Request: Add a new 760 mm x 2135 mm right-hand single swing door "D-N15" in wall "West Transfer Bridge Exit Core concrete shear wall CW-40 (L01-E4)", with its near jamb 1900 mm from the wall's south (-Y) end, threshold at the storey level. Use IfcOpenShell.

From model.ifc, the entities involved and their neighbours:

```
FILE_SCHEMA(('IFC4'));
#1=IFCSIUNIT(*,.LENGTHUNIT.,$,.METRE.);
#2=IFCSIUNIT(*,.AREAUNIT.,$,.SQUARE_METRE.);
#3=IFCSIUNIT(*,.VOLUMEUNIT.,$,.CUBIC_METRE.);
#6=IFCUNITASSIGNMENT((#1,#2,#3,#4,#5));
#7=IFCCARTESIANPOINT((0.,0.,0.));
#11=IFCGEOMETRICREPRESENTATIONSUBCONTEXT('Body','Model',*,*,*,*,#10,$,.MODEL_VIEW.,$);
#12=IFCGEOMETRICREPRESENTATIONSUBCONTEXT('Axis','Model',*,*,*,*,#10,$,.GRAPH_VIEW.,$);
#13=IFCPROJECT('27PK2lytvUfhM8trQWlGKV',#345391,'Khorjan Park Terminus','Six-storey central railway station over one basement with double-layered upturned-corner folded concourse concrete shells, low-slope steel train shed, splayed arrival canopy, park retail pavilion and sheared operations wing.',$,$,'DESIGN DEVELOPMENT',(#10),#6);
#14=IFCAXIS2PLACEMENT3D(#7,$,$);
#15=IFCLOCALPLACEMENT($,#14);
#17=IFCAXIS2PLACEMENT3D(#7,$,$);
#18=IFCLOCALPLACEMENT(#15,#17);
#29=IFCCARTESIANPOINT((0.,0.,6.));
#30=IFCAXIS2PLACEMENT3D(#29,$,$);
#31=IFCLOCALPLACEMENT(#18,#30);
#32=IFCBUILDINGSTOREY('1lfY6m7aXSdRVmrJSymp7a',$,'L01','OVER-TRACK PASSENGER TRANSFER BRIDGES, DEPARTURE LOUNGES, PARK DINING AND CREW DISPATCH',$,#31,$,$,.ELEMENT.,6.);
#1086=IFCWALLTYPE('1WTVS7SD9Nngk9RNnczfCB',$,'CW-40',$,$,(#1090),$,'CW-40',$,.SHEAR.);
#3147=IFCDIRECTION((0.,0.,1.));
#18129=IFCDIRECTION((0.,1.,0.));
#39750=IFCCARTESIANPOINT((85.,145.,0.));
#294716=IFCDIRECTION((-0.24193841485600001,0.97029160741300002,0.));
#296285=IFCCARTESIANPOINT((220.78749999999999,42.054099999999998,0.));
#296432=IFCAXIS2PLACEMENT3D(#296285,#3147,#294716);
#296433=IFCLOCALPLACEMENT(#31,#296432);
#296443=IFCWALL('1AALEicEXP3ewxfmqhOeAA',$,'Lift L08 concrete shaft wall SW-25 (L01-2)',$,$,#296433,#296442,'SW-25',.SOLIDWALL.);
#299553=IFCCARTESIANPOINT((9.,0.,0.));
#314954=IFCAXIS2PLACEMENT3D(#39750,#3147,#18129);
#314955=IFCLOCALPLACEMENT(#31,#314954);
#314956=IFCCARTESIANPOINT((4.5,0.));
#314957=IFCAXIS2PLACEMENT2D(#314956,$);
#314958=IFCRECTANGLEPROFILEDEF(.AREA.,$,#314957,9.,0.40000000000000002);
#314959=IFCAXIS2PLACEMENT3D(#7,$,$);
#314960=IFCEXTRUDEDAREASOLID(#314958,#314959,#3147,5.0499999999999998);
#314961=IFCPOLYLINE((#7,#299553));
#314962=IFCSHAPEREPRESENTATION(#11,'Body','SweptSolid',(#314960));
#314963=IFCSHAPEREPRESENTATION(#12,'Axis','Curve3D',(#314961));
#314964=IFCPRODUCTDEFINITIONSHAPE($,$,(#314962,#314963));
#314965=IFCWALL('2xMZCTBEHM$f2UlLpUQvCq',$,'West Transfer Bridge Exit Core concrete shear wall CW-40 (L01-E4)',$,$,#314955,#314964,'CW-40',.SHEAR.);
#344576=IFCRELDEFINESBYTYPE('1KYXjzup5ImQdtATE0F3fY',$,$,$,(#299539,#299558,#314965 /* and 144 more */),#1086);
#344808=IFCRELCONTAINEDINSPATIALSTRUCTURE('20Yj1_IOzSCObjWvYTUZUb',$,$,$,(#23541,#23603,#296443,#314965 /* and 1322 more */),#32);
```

```python
import numpy as np
import ifcopenshell
import ifcopenshell.api.feature
import ifcopenshell.api.geometry
import ifcopenshell.api.root
import ifcopenshell.api.spatial
import ifcopenshell.geom
import ifcopenshell.util.element
import ifcopenshell.util.placement
import ifcopenshell.util.representation
import ifcopenshell.util.shape
import ifcopenshell.util.unit

model = ifcopenshell.open("model.ifc")
unit_scale = ifcopenshell.util.unit.calculate_unit_scale(model)
settings = ifcopenshell.geom.settings()


def volume(element):
    """Net volume in cubic metres, openings subtracted."""
    shape = ifcopenshell.geom.create_shape(settings, element)
    return ifcopenshell.util.shape.get_volume(shape.geometry)


wall = model.by_guid("2xMZCTBEHM$f2UlLpUQvCq")
storey = ifcopenshell.util.element.get_container(wall, ifc_class="IfcBuildingStorey")
context = ifcopenshell.util.representation.get_context(model, "Model", "Body", "MODEL_VIEW")
before = volume(wall)

width, height, from_end, sill = 0.76, 2.135, 1.9, 0.0  # metres

# The wall runs along its own X axis, and the end named is its -X end.
wall_shape = ifcopenshell.geom.create_shape(settings, wall)
x, y, z = ifcopenshell.util.shape.get_vertices(wall_shape.geometry).T
start = x.min() + from_end
face, thickness = float(y.min()), float(y.max() - y.min())
wall_matrix = ifcopenshell.util.placement.get_local_placement(wall.ObjectPlacement)
level = ifcopenshell.util.placement.get_local_placement(storey.ObjectPlacement)[2, 3]


def in_wall(x, y):
    """Placement at x, y metres in the wall's axes, at sill height."""
    matrix = wall_matrix.copy()
    matrix[:, 3] = wall_matrix @ np.array([x / unit_scale, y / unit_scale, 0.0, 1.0])
    matrix[2, 3] = level + sill / unit_scale
    return matrix


# Opening: a box that overshoots both wall faces by 50 mm.
opening = ifcopenshell.api.root.create_entity(model, ifc_class="IfcOpeningElement", predefined_type="OPENING")
box = ifcopenshell.api.geometry.add_wall_representation(
    model, context=context, length=width, height=height, thickness=thickness + 0.1
)
ifcopenshell.api.geometry.assign_representation(model, product=opening, representation=box)
ifcopenshell.api.geometry.edit_object_placement(model, product=opening, matrix=in_wall(start, face - 0.05), is_si=False)
ifcopenshell.api.feature.add_feature(model, feature=opening, element=wall)

door = ifcopenshell.api.root.create_entity(model, ifc_class="IfcDoor", name="D-N15", predefined_type="DOOR")
door.OverallWidth, door.OverallHeight = width / unit_scale, height / unit_scale
door.OperationType = "SINGLE_SWING_RIGHT"
body = ifcopenshell.api.geometry.add_door_representation(
    model,
    context=context,
    overall_width=door.OverallWidth,
    overall_height=door.OverallHeight,
    operation_type="SINGLE_SWING_RIGHT",
    lining_properties={"LiningDepth": thickness / unit_scale, "ThresholdDepth": thickness / unit_scale},
)
ifcopenshell.api.geometry.assign_representation(model, product=door, representation=body)
ifcopenshell.api.spatial.assign_container(model, products=[door], relating_structure=storey)
ifcopenshell.api.feature.add_filling(model, opening=opening, element=door)

# The lining spans the wall, so the door starts at the wall face.
ifcopenshell.api.geometry.edit_object_placement(model, product=door, matrix=in_wall(start, face), is_si=False)

after = volume(wall)

print(f"wall volume {before:.3f} -> {after:.3f} m3")

model.write("model_updated.ifc")
```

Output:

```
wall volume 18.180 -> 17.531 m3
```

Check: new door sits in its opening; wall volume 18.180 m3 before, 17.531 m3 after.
